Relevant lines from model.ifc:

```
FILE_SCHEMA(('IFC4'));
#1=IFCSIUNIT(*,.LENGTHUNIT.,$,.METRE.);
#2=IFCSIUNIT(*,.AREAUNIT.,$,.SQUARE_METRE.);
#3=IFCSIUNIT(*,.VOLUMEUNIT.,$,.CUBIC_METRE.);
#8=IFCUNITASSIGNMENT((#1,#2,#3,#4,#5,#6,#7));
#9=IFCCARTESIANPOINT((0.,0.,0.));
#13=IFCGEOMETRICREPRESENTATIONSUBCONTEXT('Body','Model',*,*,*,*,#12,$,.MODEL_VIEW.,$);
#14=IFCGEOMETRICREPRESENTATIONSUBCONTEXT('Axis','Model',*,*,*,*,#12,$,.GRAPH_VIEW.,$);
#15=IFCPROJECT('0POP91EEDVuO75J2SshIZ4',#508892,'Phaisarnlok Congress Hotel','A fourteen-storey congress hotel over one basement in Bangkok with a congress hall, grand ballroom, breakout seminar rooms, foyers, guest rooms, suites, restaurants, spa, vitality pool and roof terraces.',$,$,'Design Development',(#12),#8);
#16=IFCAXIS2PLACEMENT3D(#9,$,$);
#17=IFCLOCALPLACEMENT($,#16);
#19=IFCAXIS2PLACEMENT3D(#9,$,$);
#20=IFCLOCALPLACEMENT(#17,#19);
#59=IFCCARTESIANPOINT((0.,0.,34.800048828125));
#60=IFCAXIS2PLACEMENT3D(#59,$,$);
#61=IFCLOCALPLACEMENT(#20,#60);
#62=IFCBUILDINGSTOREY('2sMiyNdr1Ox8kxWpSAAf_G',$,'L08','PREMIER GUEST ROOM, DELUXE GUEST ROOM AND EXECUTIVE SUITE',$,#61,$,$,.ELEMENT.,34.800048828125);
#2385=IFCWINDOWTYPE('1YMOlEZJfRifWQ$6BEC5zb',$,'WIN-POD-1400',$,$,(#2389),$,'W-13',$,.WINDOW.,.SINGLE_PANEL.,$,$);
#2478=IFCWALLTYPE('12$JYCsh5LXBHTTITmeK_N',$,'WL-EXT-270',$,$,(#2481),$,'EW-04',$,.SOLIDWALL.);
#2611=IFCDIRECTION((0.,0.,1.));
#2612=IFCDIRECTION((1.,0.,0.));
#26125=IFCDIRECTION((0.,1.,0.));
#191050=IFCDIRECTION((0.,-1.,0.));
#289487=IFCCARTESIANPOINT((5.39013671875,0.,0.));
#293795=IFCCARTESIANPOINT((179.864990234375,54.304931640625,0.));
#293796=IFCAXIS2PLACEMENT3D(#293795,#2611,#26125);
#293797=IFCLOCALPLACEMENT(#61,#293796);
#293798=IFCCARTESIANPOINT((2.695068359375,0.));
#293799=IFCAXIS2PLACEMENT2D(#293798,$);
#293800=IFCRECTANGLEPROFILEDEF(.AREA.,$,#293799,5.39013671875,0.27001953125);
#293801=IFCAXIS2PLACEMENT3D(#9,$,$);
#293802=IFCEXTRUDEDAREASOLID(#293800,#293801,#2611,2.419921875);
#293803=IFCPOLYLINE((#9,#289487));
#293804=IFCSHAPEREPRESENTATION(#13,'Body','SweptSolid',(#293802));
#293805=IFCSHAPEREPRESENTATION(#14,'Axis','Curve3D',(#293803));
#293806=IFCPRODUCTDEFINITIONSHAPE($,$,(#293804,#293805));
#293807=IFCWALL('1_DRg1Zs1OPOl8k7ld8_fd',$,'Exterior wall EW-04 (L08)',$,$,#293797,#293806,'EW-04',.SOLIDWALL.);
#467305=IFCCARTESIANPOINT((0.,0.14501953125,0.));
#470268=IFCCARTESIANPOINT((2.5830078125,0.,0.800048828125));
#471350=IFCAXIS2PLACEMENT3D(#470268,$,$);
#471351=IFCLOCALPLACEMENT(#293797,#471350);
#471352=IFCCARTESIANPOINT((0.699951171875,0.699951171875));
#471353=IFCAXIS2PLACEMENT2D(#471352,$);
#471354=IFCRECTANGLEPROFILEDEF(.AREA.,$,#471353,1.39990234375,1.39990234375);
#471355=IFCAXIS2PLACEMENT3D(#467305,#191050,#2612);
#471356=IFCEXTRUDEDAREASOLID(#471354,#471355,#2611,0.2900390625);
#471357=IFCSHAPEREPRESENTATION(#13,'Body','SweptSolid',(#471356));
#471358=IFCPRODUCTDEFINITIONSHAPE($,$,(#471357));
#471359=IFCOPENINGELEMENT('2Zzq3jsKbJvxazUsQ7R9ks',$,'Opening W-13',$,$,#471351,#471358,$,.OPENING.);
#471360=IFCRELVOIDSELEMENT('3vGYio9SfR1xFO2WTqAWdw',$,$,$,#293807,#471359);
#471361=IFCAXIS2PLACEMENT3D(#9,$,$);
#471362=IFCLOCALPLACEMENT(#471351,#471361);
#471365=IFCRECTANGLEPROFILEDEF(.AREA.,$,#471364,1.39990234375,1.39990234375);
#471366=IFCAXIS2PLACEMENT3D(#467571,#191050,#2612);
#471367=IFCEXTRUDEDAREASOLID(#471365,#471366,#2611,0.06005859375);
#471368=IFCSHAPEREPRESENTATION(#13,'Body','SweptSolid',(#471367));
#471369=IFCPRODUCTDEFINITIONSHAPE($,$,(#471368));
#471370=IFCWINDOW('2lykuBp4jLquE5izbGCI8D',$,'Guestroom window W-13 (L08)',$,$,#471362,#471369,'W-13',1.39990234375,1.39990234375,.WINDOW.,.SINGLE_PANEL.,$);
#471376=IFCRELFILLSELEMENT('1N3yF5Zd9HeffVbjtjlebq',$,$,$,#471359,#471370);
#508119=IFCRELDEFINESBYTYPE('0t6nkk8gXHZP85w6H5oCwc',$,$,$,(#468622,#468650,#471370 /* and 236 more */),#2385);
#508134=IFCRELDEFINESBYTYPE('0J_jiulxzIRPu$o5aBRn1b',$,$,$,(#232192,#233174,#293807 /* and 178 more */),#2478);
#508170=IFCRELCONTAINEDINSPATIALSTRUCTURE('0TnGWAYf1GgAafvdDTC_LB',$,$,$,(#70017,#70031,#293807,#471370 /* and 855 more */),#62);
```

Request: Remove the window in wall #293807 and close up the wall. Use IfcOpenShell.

```python
import ifcopenshell
import ifcopenshell.api.feature
import ifcopenshell.api.root
import ifcopenshell.geom
import ifcopenshell.util.shape

model = ifcopenshell.open("model.ifc")
settings = ifcopenshell.geom.settings()


def volume(element):
    """Net volume in cubic metres, openings subtracted."""
    shape = ifcopenshell.geom.create_shape(settings, element)
    return ifcopenshell.util.shape.get_volume(shape.geometry)


window = model.by_id(471370)
opening = window.FillsVoids[0].RelatingOpeningElement
wall = opening.VoidsElements[0].RelatingBuildingElement
before = volume(wall)

ifcopenshell.api.root.remove_product(model, product=window)
ifcopenshell.api.feature.remove_feature(model, feature=opening)

after = volume(wall)

print(f"wall volume {before:.3f} -> {after:.3f} m3")

model.write("model_updated.ifc")
```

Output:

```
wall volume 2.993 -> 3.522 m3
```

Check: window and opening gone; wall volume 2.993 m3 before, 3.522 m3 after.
